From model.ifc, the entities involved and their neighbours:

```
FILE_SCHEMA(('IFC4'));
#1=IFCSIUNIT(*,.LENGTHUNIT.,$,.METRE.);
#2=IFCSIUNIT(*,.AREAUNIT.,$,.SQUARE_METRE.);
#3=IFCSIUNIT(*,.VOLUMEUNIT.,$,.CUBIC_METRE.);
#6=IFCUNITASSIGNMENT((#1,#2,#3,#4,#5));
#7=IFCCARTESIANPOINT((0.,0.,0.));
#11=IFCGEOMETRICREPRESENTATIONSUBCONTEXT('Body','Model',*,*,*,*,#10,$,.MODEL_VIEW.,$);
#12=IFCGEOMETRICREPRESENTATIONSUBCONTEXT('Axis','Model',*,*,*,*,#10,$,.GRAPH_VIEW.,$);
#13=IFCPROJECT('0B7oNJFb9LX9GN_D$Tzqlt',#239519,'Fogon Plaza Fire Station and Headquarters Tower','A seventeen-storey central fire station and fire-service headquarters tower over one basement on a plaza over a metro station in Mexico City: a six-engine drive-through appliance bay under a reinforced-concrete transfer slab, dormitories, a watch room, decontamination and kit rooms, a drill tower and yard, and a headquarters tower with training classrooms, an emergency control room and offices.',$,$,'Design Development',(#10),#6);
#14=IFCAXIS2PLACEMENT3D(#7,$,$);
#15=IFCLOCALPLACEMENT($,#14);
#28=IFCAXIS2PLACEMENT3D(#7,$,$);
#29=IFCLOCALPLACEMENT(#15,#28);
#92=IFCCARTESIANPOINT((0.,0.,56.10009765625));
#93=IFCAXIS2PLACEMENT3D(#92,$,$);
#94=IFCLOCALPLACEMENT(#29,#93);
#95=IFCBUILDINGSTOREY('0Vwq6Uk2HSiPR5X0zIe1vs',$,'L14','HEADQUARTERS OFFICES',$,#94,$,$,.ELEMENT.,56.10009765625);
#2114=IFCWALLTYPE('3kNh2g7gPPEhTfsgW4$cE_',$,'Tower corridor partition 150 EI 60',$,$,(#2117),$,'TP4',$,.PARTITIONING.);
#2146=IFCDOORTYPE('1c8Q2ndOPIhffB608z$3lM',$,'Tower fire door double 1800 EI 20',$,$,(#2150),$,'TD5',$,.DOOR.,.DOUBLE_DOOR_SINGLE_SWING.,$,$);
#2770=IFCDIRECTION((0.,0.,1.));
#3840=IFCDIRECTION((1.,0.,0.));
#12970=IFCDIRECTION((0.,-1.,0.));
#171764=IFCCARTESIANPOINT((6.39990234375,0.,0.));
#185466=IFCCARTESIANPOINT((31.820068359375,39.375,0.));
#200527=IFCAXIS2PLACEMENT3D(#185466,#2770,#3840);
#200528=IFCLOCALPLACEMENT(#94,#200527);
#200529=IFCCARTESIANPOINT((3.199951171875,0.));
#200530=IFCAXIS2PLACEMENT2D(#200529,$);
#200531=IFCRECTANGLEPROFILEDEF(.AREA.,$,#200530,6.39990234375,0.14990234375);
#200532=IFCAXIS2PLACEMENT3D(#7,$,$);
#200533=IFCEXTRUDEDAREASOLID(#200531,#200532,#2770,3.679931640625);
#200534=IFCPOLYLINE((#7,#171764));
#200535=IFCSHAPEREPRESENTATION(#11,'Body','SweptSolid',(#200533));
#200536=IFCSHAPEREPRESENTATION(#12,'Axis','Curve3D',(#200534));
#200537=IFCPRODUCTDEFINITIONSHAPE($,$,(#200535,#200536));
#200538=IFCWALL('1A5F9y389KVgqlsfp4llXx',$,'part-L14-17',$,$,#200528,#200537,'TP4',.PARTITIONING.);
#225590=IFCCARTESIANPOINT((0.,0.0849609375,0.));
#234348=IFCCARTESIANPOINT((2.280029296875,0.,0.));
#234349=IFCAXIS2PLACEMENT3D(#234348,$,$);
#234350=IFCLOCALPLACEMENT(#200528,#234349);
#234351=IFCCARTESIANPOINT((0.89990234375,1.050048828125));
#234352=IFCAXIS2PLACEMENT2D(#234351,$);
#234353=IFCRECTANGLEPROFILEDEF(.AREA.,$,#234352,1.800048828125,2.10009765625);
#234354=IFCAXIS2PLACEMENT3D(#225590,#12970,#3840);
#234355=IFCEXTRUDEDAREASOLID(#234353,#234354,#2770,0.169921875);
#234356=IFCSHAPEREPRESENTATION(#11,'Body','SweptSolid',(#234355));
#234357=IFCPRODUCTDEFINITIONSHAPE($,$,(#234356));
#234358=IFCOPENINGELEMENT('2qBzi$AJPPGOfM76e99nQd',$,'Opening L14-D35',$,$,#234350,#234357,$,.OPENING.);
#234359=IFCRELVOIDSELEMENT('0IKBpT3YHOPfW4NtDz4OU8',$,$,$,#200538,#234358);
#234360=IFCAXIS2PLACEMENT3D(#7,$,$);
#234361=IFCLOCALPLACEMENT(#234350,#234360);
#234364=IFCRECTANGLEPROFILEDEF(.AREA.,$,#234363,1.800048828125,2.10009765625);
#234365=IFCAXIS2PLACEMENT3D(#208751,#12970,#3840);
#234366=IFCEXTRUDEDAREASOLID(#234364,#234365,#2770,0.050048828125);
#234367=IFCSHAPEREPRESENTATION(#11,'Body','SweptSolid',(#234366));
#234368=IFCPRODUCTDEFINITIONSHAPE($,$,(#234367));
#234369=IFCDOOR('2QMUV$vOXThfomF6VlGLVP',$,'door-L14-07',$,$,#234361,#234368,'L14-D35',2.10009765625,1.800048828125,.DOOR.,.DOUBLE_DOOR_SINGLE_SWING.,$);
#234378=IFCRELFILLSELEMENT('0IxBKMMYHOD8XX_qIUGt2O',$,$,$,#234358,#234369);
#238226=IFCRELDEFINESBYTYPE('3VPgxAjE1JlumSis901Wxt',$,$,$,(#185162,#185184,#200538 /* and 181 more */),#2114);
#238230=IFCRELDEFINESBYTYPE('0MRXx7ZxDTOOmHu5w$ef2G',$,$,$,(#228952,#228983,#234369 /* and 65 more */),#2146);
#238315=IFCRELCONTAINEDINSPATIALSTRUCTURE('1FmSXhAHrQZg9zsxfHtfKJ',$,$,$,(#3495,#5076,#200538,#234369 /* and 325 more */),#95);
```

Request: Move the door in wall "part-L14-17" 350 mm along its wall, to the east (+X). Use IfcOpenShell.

```python
import ifcopenshell
import ifcopenshell.api.geometry
import ifcopenshell.util.placement
import ifcopenshell.util.unit

model = ifcopenshell.open("model.ifc")
unit_scale = ifcopenshell.util.unit.calculate_unit_scale(model)

door = model.by_guid("2QMUV$vOXThfomF6VlGLVP")
opening = door.FillsVoids[0].RelatingOpeningElement
wall = opening.VoidsElements[0].RelatingBuildingElement

wall_matrix = ifcopenshell.util.placement.get_local_placement(wall.ObjectPlacement)
shift = wall_matrix[:3, 0] * 0.35 / unit_scale
before = ifcopenshell.util.placement.get_local_placement(door.ObjectPlacement)[:3, 3].copy()

# The door is placed relative to its opening, so it follows when the opening moves.
matrix = ifcopenshell.util.placement.get_local_placement(opening.ObjectPlacement)
matrix[:3, 3] += shift
ifcopenshell.api.geometry.edit_object_placement(
    model, product=opening, matrix=matrix, is_si=False, should_transform_children=True
)

after = ifcopenshell.util.placement.get_local_placement(door.ObjectPlacement)[:3, 3]
print("door moved by", (after - before).round(3) + 0.0)

model.write("model_updated.ifc")
```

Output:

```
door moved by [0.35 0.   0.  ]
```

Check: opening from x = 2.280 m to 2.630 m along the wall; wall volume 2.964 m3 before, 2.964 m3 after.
